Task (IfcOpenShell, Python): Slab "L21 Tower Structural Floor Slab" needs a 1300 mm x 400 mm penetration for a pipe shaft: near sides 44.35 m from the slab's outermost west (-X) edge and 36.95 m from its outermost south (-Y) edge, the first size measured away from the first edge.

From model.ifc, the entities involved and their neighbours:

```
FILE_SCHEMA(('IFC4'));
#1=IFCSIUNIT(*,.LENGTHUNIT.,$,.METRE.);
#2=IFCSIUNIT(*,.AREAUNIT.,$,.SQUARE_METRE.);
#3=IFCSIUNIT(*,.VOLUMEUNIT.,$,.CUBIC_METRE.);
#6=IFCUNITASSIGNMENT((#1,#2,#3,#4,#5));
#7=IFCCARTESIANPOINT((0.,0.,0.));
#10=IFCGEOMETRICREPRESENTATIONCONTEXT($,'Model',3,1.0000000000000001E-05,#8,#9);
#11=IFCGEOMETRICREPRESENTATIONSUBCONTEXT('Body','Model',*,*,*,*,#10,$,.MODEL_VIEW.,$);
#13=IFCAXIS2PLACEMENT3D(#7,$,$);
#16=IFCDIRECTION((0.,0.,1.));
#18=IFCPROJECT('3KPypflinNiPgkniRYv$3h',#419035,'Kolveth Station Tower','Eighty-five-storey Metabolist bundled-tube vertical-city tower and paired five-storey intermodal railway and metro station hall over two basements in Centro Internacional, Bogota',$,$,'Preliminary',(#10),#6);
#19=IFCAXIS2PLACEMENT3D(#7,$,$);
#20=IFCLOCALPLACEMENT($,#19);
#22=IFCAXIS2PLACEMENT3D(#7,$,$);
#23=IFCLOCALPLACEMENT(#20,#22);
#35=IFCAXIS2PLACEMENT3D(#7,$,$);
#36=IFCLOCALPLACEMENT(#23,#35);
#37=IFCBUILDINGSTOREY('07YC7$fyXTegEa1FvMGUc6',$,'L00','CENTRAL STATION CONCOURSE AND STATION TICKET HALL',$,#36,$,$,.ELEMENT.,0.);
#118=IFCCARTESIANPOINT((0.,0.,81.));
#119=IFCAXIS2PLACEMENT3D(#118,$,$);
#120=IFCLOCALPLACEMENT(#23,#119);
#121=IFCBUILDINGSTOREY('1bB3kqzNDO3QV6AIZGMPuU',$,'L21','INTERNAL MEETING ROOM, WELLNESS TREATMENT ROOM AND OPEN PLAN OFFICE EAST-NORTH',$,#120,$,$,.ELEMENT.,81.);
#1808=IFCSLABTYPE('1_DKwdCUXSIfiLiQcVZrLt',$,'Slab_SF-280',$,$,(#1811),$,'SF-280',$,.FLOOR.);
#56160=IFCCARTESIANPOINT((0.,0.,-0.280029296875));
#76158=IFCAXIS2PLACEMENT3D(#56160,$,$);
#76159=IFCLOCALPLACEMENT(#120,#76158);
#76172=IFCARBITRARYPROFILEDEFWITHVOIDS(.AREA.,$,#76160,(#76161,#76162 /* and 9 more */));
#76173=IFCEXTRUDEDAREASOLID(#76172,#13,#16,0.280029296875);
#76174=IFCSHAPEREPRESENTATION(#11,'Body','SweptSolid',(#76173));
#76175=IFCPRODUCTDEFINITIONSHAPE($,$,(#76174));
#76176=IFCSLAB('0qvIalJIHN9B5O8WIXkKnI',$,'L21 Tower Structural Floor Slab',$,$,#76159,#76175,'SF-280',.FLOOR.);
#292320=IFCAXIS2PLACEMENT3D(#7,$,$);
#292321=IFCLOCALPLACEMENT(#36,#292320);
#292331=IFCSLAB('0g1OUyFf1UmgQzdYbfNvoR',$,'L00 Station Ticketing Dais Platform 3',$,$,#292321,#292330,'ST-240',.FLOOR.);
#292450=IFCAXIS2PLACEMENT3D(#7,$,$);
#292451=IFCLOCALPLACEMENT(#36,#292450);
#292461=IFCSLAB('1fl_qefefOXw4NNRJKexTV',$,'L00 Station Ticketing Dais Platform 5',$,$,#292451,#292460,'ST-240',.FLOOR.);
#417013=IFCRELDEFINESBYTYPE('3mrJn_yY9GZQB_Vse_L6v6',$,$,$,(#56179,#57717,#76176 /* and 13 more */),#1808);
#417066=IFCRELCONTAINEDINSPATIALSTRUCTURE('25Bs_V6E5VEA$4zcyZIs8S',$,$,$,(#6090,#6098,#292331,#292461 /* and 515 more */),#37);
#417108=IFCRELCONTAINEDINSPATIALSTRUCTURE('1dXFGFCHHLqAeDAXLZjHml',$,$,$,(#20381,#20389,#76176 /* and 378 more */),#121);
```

```python
import numpy as np
import ifcopenshell
import ifcopenshell.api.feature
import ifcopenshell.api.geometry
import ifcopenshell.api.root
import ifcopenshell.geom
import ifcopenshell.util.placement
import ifcopenshell.util.representation
import ifcopenshell.util.shape
import ifcopenshell.util.unit

model = ifcopenshell.open("model.ifc")
unit_scale = ifcopenshell.util.unit.calculate_unit_scale(model)
settings = ifcopenshell.geom.settings()


def volume(element):
    """Net volume in cubic metres, openings subtracted."""
    shape = ifcopenshell.geom.create_shape(settings, element)
    return ifcopenshell.util.shape.get_volume(shape.geometry)


slab = model.by_id(76176)
before = volume(slab)

# Extent in the slab's own axes, in metres. The edges named are its -X and -Y sides.
slab_shape = ifcopenshell.geom.create_shape(settings, slab)
vertices = ifcopenshell.util.shape.get_vertices(slab_shape.geometry)
x_min, y_min, bottom = vertices.min(axis=0)
top = vertices[:, 2].max()

opening = ifcopenshell.api.root.create_entity(model, ifc_class="IfcOpeningElement", name="Pipe shaft opening", predefined_type="OPENING")
context = ifcopenshell.util.representation.get_context(model, "Model", "Body", "MODEL_VIEW")
width, depth = 1.3, 0.4
outline = [(0.0, 0.0), (width, 0.0), (width, depth), (0.0, depth), (0.0, 0.0)]
# Overshoot both faces by 50 mm so the cut is clean.
shape = ifcopenshell.api.geometry.add_slab_representation(
    model, context=context, depth=top - bottom + 0.1, polyline=outline
)
ifcopenshell.api.geometry.assign_representation(model, product=opening, representation=shape)

matrix = ifcopenshell.util.placement.get_local_placement(slab.ObjectPlacement)
matrix[:, 3] = matrix @ np.append(np.array([x_min + 44.35, y_min + 36.95, bottom - 0.05]) / unit_scale, 1.0)
ifcopenshell.api.geometry.edit_object_placement(model, product=opening, matrix=matrix, is_si=False)
ifcopenshell.api.feature.add_feature(model, feature=opening, element=slab)

after = volume(slab)

print(f"slab volume {before:.3f} -> {after:.3f} m3")

model.write("model_updated.ifc")
```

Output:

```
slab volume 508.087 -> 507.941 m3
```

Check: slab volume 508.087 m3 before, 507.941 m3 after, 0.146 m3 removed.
